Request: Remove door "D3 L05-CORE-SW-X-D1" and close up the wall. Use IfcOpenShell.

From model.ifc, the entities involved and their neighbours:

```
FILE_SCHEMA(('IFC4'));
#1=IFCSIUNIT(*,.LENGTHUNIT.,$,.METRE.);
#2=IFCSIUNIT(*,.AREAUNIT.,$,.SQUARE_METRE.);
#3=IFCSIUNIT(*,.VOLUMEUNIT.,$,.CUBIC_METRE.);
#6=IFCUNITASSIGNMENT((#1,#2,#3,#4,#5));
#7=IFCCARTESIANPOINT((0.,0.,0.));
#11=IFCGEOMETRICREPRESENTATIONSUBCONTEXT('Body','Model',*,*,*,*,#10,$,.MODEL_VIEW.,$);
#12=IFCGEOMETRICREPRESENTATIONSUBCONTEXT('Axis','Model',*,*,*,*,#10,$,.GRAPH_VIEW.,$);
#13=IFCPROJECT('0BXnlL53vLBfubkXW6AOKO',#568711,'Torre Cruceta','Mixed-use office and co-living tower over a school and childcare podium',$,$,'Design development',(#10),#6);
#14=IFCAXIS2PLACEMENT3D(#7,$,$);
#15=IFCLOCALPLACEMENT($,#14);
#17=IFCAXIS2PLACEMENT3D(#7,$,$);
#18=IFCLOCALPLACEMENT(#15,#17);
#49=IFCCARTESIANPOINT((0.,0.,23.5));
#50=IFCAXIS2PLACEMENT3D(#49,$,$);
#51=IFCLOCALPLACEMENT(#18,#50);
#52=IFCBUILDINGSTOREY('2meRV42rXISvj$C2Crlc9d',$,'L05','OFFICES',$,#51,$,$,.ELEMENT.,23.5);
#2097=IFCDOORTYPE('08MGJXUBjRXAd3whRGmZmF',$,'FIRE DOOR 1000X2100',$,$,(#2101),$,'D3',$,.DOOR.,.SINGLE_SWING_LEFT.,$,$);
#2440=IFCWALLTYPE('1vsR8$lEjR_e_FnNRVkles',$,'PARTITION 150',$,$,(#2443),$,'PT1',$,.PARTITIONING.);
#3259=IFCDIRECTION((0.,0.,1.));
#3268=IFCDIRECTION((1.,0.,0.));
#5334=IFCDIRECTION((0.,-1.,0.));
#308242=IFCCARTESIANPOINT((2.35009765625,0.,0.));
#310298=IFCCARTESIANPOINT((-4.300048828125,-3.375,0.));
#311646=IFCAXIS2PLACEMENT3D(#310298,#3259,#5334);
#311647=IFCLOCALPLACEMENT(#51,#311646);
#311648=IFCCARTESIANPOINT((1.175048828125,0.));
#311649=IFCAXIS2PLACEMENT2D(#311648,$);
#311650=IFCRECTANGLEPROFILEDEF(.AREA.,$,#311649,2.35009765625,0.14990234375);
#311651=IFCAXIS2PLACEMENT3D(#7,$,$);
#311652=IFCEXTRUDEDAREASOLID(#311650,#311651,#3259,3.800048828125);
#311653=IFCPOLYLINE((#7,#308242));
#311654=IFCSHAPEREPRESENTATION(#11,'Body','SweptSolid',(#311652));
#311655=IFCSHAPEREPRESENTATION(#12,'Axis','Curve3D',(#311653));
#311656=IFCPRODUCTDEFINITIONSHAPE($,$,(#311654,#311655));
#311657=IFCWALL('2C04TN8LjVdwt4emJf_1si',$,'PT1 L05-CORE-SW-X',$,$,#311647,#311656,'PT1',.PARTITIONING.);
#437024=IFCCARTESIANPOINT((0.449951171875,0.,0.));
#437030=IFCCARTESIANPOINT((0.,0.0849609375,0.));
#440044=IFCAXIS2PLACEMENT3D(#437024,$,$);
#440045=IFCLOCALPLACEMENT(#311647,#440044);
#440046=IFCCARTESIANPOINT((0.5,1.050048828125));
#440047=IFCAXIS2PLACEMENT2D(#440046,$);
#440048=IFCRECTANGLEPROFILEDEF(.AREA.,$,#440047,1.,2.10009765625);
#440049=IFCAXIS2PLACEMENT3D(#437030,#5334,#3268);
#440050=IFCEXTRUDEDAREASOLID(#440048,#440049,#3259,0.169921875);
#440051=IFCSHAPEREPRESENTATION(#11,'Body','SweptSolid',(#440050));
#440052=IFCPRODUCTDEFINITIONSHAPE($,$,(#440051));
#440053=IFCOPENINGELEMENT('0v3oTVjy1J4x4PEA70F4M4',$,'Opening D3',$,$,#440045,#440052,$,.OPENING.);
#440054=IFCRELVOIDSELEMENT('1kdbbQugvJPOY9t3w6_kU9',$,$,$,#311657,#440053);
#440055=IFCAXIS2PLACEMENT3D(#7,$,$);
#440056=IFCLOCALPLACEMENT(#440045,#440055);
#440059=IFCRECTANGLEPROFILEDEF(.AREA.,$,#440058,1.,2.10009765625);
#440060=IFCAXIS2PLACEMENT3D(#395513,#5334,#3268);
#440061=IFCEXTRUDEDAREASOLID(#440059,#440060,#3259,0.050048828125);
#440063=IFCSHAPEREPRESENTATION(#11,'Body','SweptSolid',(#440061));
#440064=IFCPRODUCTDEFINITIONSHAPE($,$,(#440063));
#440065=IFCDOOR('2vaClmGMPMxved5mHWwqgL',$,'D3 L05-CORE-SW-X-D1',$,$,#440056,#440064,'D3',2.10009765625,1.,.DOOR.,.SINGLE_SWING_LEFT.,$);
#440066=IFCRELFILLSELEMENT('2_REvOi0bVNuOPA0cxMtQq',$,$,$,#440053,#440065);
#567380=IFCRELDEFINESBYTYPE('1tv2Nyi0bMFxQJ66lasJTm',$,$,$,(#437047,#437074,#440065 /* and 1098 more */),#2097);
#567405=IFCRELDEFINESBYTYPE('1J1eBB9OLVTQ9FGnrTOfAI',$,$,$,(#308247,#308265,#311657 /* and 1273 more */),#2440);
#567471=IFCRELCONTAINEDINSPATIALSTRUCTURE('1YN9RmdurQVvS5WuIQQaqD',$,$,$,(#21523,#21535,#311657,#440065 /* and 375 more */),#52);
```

```python
import ifcopenshell
import ifcopenshell.api.feature
import ifcopenshell.api.root
import ifcopenshell.geom
import ifcopenshell.util.shape

model = ifcopenshell.open("model.ifc")
settings = ifcopenshell.geom.settings()


def volume(element):
    """Net volume in cubic metres, openings subtracted."""
    shape = ifcopenshell.geom.create_shape(settings, element)
    return ifcopenshell.util.shape.get_volume(shape.geometry)


door = model.by_guid("2vaClmGMPMxved5mHWwqgL")
opening = door.FillsVoids[0].RelatingOpeningElement
wall = opening.VoidsElements[0].RelatingBuildingElement
before = volume(wall)

ifcopenshell.api.root.remove_product(model, product=door)
ifcopenshell.api.feature.remove_feature(model, feature=opening)

after = volume(wall)

print(f"wall volume {before:.3f} -> {after:.3f} m3")

model.write("model_updated.ifc")
```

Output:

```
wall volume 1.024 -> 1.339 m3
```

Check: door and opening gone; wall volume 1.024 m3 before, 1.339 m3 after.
